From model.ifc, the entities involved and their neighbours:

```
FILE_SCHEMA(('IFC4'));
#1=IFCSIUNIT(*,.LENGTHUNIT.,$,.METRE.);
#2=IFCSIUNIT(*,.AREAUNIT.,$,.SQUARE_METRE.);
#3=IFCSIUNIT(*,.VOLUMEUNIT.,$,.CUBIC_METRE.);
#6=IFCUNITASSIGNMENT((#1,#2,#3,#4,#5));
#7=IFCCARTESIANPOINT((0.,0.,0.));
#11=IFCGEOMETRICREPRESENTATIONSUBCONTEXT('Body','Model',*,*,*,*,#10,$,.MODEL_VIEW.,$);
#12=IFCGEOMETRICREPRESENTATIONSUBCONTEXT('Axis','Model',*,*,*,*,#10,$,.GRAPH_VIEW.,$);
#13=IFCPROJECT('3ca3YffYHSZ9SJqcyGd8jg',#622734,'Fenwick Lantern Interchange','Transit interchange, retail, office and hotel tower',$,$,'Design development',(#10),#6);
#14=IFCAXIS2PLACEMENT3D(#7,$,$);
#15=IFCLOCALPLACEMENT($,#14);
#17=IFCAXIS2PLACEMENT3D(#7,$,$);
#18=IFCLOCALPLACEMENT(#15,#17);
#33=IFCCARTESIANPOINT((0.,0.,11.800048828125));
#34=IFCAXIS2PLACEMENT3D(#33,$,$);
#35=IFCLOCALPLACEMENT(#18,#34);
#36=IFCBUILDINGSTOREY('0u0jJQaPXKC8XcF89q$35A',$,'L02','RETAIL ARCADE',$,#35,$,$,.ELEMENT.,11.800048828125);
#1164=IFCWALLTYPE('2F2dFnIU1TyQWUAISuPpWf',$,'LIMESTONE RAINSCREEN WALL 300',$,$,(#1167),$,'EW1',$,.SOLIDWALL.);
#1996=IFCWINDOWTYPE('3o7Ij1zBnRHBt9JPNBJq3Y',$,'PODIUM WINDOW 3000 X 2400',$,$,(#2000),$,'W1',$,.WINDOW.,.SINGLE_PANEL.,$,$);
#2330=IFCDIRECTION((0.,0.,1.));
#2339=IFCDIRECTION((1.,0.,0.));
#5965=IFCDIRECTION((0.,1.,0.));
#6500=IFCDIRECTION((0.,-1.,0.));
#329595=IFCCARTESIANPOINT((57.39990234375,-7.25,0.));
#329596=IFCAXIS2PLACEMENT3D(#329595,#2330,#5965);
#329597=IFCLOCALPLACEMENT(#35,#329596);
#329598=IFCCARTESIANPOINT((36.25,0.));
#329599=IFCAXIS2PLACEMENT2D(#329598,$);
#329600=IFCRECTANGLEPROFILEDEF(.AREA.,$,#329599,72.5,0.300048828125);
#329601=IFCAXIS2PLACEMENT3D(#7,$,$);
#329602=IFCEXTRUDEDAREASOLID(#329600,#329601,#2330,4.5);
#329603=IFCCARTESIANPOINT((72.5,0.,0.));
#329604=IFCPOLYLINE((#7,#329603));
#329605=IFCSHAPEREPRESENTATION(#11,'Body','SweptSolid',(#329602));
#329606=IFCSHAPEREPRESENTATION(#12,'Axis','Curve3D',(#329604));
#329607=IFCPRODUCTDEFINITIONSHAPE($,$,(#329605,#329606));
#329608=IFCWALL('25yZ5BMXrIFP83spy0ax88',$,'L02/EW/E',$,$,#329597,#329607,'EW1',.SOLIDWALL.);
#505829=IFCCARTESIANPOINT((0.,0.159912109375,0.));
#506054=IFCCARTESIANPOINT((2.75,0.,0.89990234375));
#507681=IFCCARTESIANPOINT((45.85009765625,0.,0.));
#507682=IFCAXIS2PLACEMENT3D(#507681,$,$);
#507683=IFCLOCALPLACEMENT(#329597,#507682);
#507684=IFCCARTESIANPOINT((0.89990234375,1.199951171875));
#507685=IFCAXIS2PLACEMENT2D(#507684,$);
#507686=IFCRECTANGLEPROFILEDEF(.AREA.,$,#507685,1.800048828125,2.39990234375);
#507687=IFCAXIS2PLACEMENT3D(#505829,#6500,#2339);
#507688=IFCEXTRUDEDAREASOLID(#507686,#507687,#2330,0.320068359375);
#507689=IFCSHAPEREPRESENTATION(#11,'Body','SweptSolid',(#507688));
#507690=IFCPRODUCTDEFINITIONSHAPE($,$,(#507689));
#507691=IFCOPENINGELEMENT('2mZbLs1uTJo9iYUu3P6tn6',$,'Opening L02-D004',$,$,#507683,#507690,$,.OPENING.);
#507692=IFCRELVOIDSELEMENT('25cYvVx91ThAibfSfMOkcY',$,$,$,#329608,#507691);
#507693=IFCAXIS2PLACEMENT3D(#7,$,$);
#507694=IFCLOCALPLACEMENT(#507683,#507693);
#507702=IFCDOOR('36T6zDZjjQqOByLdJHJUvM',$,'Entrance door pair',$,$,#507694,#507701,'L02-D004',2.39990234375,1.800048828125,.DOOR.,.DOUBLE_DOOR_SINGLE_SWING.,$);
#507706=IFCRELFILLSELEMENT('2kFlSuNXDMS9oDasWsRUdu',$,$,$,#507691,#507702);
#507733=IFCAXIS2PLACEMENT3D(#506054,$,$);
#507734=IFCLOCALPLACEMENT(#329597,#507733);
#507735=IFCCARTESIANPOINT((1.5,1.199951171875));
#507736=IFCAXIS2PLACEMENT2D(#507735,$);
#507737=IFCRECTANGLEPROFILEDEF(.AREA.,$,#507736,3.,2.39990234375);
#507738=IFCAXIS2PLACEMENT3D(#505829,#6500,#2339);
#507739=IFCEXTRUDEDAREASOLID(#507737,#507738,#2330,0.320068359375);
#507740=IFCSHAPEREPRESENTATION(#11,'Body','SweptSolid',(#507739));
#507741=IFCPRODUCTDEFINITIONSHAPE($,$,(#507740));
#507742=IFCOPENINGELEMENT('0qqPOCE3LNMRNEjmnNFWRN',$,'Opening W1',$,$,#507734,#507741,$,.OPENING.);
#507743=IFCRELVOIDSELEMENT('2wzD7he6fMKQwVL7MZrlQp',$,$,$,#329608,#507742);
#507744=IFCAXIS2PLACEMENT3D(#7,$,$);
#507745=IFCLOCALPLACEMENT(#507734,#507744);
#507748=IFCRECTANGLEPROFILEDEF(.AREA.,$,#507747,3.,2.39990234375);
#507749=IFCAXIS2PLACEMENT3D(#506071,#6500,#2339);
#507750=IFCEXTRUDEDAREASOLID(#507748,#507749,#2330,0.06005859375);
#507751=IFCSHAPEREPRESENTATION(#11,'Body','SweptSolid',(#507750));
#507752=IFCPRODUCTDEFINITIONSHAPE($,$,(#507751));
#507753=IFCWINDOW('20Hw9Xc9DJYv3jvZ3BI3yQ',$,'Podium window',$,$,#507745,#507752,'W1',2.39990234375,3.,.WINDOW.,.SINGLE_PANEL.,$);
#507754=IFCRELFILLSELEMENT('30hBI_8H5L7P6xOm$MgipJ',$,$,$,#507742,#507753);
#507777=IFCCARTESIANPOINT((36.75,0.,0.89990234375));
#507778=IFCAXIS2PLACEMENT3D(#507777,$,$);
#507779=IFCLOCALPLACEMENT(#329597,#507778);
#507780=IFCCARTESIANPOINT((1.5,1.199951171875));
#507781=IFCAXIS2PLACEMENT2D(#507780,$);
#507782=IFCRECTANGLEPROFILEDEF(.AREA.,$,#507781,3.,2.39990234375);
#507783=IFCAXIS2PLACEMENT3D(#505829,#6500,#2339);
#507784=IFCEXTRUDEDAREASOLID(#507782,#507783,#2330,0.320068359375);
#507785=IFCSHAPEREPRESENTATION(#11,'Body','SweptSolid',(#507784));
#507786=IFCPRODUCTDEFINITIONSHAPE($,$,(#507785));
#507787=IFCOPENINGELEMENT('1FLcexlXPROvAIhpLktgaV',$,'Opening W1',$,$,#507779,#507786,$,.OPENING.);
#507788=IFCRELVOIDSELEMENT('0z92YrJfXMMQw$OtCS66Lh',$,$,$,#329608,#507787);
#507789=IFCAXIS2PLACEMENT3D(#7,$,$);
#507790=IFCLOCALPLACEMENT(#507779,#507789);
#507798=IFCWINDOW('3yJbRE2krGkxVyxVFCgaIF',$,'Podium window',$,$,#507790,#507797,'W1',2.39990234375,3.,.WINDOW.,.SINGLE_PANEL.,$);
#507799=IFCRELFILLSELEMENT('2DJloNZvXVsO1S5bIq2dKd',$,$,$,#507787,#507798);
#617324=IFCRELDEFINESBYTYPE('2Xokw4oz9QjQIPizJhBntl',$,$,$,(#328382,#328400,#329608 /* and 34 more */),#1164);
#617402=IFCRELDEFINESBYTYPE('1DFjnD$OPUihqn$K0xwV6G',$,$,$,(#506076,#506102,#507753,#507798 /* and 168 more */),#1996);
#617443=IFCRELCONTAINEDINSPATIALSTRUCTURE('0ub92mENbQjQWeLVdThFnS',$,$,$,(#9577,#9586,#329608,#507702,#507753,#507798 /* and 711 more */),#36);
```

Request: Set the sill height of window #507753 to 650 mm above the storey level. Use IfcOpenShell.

```python
import numpy as np
import ifcopenshell
import ifcopenshell.api.geometry
import ifcopenshell.geom
import ifcopenshell.util.element
import ifcopenshell.util.placement
import ifcopenshell.util.shape
import ifcopenshell.util.unit

model = ifcopenshell.open("model.ifc")
unit_scale = ifcopenshell.util.unit.calculate_unit_scale(model)

window = model.by_guid("20Hw9Xc9DJYv3jvZ3BI3yQ")
opening = window.FillsVoids[0].RelatingOpeningElement
storey = ifcopenshell.util.element.get_container(window, ifc_class="IfcBuildingStorey")
level = ifcopenshell.util.placement.get_local_placement(storey.ObjectPlacement)[2, 3]

# The opening's origin need not be at the sill, so measure its lowest point.
shape = ifcopenshell.geom.create_shape(ifcopenshell.geom.settings(), opening)
bottom = ifcopenshell.util.shape.get_shape_bottom_elevation(shape, shape.geometry) / unit_scale
dz = level + 0.65 / unit_scale - bottom

shift = np.array([0.0, 0.0, dz])
# The window is placed relative to its opening, so it follows when the opening moves.
matrix = ifcopenshell.util.placement.get_local_placement(opening.ObjectPlacement)
matrix[:3, 3] += shift
ifcopenshell.api.geometry.edit_object_placement(
    model, product=opening, matrix=matrix, is_si=False, should_transform_children=True
)

print(f"moved by {dz * unit_scale:+.3f} m")

model.write("model_rev.ifc")
```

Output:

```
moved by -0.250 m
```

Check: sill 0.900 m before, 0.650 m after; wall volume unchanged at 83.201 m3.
